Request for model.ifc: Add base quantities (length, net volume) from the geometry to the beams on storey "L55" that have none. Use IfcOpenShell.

First a look at what the model holds.

```python
import ifcopenshell
import ifcopenshell.util.element
import ifcopenshell.util.unit

model = ifcopenshell.open("model.ifc")
print(model.schema)
for unit_type in ("LENGTHUNIT", "AREAUNIT", "VOLUMEUNIT"):
    print(unit_type, ifcopenshell.util.unit.calculate_unit_scale(model, unit_type))
storey = next(s for s in model.by_type("IfcBuildingStorey") if s.Name == "L55")
beams = [e for e in ifcopenshell.util.element.get_decomposition(storey) if e.is_a("IfcBeam")]
for e in sorted(beams, key=lambda e: e.id()):
    print(e.id(), e.is_a(), e.Name, list(ifcopenshell.util.element.get_psets(e, qtos_only=True)), sep=" | ")
```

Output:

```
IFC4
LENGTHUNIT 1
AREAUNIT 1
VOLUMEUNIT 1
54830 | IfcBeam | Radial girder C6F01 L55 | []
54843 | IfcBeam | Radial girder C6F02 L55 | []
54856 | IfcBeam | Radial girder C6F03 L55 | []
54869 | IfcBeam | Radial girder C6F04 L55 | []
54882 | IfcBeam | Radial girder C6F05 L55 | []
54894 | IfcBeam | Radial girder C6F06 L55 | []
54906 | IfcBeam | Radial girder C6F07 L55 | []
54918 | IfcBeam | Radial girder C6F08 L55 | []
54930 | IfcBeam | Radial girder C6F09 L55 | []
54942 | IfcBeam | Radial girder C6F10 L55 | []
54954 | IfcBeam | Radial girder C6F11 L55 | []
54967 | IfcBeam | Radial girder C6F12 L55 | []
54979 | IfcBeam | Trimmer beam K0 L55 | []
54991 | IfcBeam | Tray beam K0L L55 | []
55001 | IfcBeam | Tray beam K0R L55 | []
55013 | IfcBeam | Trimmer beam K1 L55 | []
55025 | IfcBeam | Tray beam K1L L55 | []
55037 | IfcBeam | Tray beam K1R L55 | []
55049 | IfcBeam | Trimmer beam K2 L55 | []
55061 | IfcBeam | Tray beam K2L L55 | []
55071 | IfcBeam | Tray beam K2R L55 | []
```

```python
import ifcopenshell
import ifcopenshell.api.pset
import ifcopenshell.geom
import ifcopenshell.util.element
import ifcopenshell.util.shape
import ifcopenshell.util.unit

model = ifcopenshell.open("model.ifc")
unit_scale = ifcopenshell.util.unit.calculate_unit_scale(model)
volume_scale = ifcopenshell.util.unit.calculate_unit_scale(model, "VOLUMEUNIT")
settings = ifcopenshell.geom.settings()

storey = next(s for s in model.by_type("IfcBuildingStorey") if s.Name == "L55")
beams = [e for e in ifcopenshell.util.element.get_decomposition(storey) if e.is_a("IfcBeam")]

for e in sorted(beams, key=lambda e: e.id()):
    if ifcopenshell.util.element.get_psets(e, qtos_only=True, should_inherit=False):
        continue
    # Geometry comes back in metres, in the element's own axes.
    shape = ifcopenshell.geom.create_shape(settings, e)
    values = {
        "Length": ifcopenshell.util.shape.get_max_xyz(shape.geometry) / unit_scale,
        "NetVolume": ifcopenshell.util.shape.get_volume(shape.geometry) / volume_scale,
    }
    qto = ifcopenshell.api.pset.add_qto(model, product=e, name="Qto_BeamBaseQuantities")
    ifcopenshell.api.pset.edit_qto(model, qto=qto, properties=values)
    print(e.id(), {k: round(v, 3) for k, v in values.items()})

model.write("model_rev.ifc")
```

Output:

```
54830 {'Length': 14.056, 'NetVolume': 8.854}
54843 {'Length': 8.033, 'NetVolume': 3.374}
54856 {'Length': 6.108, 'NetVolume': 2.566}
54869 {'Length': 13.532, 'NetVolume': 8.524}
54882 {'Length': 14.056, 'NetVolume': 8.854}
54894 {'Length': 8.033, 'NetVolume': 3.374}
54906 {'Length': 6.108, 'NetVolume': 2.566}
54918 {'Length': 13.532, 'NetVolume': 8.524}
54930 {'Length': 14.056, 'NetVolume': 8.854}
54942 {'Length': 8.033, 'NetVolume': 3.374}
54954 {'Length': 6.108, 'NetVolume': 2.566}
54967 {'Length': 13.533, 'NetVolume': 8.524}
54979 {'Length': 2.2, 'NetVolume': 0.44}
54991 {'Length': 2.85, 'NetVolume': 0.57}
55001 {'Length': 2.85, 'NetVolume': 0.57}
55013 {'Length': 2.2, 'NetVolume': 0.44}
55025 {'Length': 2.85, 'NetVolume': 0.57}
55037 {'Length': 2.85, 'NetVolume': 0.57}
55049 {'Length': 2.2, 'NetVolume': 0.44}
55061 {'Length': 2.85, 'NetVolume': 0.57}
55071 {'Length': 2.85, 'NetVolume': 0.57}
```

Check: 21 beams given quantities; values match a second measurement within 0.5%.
